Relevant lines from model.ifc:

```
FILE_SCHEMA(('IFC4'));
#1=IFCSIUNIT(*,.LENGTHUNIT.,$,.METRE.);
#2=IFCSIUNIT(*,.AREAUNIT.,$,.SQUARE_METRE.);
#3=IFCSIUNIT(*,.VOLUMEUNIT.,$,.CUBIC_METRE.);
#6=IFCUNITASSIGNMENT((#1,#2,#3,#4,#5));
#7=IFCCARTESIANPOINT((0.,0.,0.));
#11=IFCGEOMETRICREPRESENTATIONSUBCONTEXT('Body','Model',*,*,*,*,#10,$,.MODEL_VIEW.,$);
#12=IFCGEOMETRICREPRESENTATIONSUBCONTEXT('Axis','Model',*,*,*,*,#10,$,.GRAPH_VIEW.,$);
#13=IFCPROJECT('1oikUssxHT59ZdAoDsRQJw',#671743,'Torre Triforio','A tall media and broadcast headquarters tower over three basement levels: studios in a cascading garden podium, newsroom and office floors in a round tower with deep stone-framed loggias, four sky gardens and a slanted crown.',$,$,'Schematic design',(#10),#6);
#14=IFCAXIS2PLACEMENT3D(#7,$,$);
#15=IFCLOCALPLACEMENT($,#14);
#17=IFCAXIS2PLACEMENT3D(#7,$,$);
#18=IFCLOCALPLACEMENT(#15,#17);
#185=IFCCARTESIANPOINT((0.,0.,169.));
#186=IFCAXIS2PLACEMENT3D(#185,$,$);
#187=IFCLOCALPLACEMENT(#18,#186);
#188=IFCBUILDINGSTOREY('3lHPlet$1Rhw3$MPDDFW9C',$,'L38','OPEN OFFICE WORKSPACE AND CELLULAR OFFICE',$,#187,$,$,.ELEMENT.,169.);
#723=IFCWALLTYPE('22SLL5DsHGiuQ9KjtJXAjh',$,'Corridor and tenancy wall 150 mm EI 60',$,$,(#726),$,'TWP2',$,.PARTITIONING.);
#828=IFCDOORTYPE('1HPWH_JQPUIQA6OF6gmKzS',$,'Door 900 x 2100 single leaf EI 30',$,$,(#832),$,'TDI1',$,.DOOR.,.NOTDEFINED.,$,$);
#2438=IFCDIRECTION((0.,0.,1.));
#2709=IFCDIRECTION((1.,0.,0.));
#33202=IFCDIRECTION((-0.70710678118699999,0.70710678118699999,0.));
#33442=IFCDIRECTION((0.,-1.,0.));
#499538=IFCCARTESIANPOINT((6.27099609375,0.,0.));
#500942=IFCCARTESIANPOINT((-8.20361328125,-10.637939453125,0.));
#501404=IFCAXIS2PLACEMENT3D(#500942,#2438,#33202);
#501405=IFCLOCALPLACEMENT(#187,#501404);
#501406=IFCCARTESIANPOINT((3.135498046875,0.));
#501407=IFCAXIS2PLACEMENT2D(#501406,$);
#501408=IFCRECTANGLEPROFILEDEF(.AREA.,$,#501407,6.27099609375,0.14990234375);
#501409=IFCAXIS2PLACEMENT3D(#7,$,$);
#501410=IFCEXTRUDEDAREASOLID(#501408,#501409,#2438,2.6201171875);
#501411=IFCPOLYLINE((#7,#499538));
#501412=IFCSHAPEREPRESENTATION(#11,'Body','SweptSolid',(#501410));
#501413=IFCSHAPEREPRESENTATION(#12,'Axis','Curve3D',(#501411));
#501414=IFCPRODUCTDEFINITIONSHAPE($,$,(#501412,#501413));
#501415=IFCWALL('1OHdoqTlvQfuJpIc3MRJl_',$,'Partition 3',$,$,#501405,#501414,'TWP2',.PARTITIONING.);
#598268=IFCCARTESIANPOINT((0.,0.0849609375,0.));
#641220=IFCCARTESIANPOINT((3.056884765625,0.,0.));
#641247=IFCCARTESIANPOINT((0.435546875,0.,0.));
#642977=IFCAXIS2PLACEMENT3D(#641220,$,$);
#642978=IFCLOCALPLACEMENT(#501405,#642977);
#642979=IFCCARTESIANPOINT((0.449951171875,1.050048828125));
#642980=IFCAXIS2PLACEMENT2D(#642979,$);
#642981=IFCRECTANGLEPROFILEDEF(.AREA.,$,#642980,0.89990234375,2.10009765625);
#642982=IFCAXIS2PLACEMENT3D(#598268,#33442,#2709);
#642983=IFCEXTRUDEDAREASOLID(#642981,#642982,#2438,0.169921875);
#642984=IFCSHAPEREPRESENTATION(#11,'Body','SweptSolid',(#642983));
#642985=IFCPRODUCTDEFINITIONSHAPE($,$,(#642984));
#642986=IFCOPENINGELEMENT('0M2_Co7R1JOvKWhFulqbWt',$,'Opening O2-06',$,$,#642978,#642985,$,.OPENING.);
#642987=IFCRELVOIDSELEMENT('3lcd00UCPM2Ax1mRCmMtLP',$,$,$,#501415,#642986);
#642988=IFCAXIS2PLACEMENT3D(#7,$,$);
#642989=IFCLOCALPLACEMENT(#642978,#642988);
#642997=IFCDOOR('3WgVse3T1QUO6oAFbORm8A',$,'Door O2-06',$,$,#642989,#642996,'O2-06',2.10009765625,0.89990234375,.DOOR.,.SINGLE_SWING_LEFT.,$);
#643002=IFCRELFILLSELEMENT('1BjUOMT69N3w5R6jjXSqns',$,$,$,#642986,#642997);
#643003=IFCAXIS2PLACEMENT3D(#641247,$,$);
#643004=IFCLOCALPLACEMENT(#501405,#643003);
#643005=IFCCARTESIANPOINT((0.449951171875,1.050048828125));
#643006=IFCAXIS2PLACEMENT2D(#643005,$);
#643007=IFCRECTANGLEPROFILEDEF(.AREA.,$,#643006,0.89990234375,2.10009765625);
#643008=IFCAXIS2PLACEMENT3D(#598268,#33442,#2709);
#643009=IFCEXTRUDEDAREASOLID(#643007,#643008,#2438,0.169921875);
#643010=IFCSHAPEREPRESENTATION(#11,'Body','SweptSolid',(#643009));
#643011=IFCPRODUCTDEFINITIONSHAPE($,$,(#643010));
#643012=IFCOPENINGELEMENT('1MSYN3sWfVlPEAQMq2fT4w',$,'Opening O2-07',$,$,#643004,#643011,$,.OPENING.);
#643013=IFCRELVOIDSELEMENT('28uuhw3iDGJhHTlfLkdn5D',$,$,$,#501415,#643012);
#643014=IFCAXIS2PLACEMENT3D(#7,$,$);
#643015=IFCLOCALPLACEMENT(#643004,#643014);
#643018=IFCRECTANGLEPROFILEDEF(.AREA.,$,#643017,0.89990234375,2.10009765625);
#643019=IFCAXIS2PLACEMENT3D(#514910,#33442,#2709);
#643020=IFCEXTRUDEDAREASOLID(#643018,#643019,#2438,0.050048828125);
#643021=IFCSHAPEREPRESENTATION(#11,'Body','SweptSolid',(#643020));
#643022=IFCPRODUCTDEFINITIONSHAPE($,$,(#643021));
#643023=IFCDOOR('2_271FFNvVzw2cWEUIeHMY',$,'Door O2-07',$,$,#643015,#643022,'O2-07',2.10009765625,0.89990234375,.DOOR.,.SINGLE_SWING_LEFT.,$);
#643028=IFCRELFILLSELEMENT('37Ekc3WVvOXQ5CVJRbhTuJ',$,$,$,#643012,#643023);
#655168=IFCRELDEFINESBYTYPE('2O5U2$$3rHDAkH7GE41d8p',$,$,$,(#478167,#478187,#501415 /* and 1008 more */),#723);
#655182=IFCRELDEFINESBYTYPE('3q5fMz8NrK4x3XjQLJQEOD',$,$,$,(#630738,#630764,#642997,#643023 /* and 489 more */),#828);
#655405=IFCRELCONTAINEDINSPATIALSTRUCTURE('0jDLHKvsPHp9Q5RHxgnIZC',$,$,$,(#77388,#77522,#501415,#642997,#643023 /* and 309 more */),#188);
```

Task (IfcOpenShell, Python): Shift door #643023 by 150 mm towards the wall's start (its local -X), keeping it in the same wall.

```python
import ifcopenshell
import ifcopenshell.api.geometry
import ifcopenshell.util.placement
import ifcopenshell.util.unit

model = ifcopenshell.open("model.ifc")
unit_scale = ifcopenshell.util.unit.calculate_unit_scale(model)

door = model.by_guid("2_271FFNvVzw2cWEUIeHMY")
opening = door.FillsVoids[0].RelatingOpeningElement
wall = opening.VoidsElements[0].RelatingBuildingElement

wall_matrix = ifcopenshell.util.placement.get_local_placement(wall.ObjectPlacement)
shift = wall_matrix[:3, 0] * -0.15 / unit_scale
before = ifcopenshell.util.placement.get_local_placement(door.ObjectPlacement)[:3, 3].copy()

# The door is placed relative to its opening, so it follows when the opening moves.
matrix = ifcopenshell.util.placement.get_local_placement(opening.ObjectPlacement)
matrix[:3, 3] += shift
ifcopenshell.api.geometry.edit_object_placement(
    model, product=opening, matrix=matrix, is_si=False, should_transform_children=True
)

after = ifcopenshell.util.placement.get_local_placement(door.ObjectPlacement)[:3, 3]
print("door moved by", (after - before).round(3) + 0.0)

model.write("model_rev.ifc")
```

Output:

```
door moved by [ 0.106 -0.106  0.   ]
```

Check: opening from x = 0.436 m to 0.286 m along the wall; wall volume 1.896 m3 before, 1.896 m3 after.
